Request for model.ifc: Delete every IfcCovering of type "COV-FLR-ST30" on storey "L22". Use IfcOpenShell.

First a look at what the model holds.

```python
import ifcopenshell
import ifcopenshell.util.element

model = ifcopenshell.open("model.ifc")
print(model.schema)
storey = next(s for s in model.by_type("IfcBuildingStorey") if s.Name == "L22")
coverings = [e for e in ifcopenshell.util.element.get_decomposition(storey) if e.is_a("IfcCovering")]
seen = {}
for e in coverings:
    element_type = ifcopenshell.util.element.get_type(e)
    name = element_type.Name if element_type not in (None, e) else None
    seen[name] = seen.get(name, 0) + 1
for name, count in sorted(seen.items(), key=str):
    print(count, "x", name)
```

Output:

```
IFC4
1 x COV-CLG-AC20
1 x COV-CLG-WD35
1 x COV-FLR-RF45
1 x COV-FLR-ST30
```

```python
import ifcopenshell
import ifcopenshell.api.root
import ifcopenshell.util.element

model = ifcopenshell.open("model.ifc")

storey = next(s for s in model.by_type("IfcBuildingStorey") if s.Name == "L22")
coverings = [e for e in ifcopenshell.util.element.get_decomposition(storey) if e.is_a("IfcCovering")]
targets = [e for e in coverings if (t := ifcopenshell.util.element.get_type(e)) not in (None, e) and t.Name == "COV-FLR-ST30"]

for e in targets:
    ifcopenshell.api.root.remove_product(model, product=e)
print(len(targets), "removed")

model.write("model-out.ifc")
```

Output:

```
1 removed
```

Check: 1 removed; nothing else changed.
